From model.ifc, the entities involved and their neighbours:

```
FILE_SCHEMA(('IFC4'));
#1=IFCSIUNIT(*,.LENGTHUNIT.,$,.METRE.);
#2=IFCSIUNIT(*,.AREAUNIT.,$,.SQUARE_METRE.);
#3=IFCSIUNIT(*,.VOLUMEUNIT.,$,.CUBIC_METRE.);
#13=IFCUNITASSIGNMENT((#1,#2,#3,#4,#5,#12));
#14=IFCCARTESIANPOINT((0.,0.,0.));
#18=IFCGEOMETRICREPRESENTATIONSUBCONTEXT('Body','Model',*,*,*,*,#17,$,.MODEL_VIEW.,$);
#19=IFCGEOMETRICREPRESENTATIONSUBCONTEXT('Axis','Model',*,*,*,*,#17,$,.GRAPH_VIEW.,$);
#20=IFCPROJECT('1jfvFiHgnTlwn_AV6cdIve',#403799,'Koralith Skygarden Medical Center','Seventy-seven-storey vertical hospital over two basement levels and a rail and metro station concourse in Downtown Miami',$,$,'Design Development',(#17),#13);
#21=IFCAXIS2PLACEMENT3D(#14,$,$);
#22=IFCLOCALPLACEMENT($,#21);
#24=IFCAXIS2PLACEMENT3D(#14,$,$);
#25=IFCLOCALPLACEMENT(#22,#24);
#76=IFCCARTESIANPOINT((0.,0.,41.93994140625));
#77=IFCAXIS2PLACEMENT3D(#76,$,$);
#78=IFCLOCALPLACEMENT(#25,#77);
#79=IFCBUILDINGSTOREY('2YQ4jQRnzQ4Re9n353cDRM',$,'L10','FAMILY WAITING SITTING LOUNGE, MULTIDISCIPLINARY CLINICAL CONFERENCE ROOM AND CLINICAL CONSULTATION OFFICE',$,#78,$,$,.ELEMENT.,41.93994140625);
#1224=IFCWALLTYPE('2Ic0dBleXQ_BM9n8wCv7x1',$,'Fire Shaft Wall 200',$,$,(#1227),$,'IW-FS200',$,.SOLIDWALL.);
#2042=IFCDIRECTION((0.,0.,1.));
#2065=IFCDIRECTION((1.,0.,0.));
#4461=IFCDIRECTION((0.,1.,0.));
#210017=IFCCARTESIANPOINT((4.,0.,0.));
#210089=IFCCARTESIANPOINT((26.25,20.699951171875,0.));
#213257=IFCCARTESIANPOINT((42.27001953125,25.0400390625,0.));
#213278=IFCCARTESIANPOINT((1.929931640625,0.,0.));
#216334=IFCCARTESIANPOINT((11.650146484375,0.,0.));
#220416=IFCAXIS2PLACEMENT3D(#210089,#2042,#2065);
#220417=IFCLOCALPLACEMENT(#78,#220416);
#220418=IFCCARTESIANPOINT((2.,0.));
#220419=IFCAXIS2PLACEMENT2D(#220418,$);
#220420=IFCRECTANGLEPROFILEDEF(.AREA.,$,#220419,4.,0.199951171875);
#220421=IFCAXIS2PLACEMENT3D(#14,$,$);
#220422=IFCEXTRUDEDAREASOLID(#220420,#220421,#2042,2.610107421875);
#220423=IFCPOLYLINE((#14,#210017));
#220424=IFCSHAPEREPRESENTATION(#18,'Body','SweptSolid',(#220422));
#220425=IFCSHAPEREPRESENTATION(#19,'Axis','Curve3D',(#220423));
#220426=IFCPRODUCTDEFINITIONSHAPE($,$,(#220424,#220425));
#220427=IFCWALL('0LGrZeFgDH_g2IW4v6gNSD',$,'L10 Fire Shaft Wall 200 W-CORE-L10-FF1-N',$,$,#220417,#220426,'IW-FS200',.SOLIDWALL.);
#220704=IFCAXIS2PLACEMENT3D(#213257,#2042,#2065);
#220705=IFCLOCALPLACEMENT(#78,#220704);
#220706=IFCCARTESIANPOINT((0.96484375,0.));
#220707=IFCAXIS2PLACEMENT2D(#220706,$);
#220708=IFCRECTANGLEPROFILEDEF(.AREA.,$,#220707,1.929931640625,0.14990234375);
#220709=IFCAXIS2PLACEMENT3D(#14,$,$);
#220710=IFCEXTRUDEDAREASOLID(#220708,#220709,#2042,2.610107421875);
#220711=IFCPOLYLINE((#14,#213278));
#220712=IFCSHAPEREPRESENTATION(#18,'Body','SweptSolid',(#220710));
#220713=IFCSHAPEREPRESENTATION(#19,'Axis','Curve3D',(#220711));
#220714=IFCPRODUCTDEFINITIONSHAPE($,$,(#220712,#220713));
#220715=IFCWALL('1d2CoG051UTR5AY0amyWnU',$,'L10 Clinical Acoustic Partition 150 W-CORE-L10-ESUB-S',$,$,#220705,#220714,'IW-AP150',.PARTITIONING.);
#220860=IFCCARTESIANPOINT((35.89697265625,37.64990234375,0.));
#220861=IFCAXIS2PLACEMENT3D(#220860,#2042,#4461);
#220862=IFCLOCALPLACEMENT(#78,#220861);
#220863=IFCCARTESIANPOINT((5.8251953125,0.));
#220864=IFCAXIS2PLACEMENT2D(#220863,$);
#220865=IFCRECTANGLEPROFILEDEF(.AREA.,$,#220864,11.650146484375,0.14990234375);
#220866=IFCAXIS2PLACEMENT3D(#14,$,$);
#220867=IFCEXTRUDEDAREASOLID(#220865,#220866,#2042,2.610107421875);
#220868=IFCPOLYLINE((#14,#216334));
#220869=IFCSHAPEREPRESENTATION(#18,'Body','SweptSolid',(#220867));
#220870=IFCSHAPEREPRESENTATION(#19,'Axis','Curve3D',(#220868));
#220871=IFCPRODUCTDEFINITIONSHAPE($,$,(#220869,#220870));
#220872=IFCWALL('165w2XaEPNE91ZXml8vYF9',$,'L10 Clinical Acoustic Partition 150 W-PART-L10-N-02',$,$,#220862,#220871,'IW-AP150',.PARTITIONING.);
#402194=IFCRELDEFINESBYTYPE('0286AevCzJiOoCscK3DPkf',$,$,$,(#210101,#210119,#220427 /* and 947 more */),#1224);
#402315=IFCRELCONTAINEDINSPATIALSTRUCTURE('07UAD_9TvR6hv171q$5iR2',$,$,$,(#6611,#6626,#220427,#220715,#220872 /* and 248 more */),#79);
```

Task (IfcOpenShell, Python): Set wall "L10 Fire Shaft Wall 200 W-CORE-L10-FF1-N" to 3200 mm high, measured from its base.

```python
import ifcopenshell
import ifcopenshell.geom
import ifcopenshell.util.representation
import ifcopenshell.util.shape
import ifcopenshell.util.unit

model = ifcopenshell.open("model.ifc")
unit_scale = ifcopenshell.util.unit.calculate_unit_scale(model)
settings = ifcopenshell.geom.settings()


def volume(element):
    """Net volume in cubic metres, openings subtracted."""
    shape = ifcopenshell.geom.create_shape(settings, element)
    return ifcopenshell.util.shape.get_volume(shape.geometry)


wall = model.by_guid("0LGrZeFgDH_g2IW4v6gNSD")
before = volume(wall)

body = ifcopenshell.util.representation.get_representation(wall, "Model", "Body")
solid = body.Items[0]
old_height = solid.Depth
solid.Depth = 3.2 / unit_scale
after = volume(wall)

print(f"height {old_height:g} -> {solid.Depth:g}, volume {before:.3f} -> {after:.3f} m3")

model.write("model_updated.ifc")
```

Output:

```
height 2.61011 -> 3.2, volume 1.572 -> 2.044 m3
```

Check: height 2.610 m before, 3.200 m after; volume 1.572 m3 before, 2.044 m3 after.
